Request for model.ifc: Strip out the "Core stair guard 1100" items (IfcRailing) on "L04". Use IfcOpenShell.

First a look at what the model holds.

```python
import ifcopenshell
import ifcopenshell.util.element

model = ifcopenshell.open("model.ifc")
print(model.schema)
storey = next(s for s in model.by_type("IfcBuildingStorey") if s.Name == "L04")
railings = [e for e in ifcopenshell.util.element.get_decomposition(storey) if e.is_a("IfcRailing")]
seen = {}
for e in railings:
    element_type = ifcopenshell.util.element.get_type(e)
    name = element_type.Name if element_type not in (None, e) else None
    seen[name] = seen.get(name, 0) + 1
for name, count in sorted(seen.items(), key=str):
    print(count, "x", name)
```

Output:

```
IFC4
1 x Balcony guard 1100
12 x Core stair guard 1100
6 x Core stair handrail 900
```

```python
import ifcopenshell
import ifcopenshell.api.root
import ifcopenshell.util.element

model = ifcopenshell.open("model.ifc")

storey = next(s for s in model.by_type("IfcBuildingStorey") if s.Name == "L04")
railings = [e for e in ifcopenshell.util.element.get_decomposition(storey) if e.is_a("IfcRailing")]
targets = [e for e in railings if (t := ifcopenshell.util.element.get_type(e)) not in (None, e) and t.Name == "Core stair guard 1100"]

for e in targets:
    ifcopenshell.api.root.remove_product(model, product=e)
print(len(targets), "removed")

model.write("model_updated.ifc")
```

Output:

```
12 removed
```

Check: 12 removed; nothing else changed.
